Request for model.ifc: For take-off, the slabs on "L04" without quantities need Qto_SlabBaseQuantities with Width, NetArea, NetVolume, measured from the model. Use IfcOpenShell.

First a look at what the model holds.

```python
import ifcopenshell
import ifcopenshell.util.element
import ifcopenshell.util.unit

model = ifcopenshell.open("model.ifc")
print(model.schema)
for unit_type in ("LENGTHUNIT", "AREAUNIT", "VOLUMEUNIT"):
    print(unit_type, ifcopenshell.util.unit.calculate_unit_scale(model, unit_type))
storey = next(s for s in model.by_type("IfcBuildingStorey") if s.Name == "L04")
slabs = [e for e in ifcopenshell.util.element.get_decomposition(storey) if e.is_a("IfcSlab")]
for e in sorted(slabs, key=lambda e: e.id()):
    print(e.id(), e.is_a(), e.Name, list(ifcopenshell.util.element.get_psets(e, qtos_only=True)), sep=" | ")
```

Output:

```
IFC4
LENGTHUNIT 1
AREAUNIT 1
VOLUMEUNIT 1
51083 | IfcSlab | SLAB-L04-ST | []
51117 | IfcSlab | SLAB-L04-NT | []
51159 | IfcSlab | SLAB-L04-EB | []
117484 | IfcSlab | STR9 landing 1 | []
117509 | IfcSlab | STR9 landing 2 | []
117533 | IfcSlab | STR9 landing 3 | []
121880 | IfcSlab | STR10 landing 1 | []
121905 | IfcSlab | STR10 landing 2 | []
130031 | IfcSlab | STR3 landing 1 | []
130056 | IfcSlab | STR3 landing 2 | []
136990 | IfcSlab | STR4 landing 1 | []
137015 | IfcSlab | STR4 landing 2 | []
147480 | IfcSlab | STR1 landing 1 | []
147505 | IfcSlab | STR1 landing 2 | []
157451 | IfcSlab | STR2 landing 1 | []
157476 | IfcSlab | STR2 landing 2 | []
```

```python
import ifcopenshell
import ifcopenshell.api.pset
import ifcopenshell.geom
import ifcopenshell.util.element
import ifcopenshell.util.shape
import ifcopenshell.util.unit

model = ifcopenshell.open("model.ifc")
unit_scale = ifcopenshell.util.unit.calculate_unit_scale(model)
area_scale = ifcopenshell.util.unit.calculate_unit_scale(model, "AREAUNIT")
volume_scale = ifcopenshell.util.unit.calculate_unit_scale(model, "VOLUMEUNIT")
settings = ifcopenshell.geom.settings()

storey = next(s for s in model.by_type("IfcBuildingStorey") if s.Name == "L04")
slabs = [e for e in ifcopenshell.util.element.get_decomposition(storey) if e.is_a("IfcSlab")]

for e in sorted(slabs, key=lambda e: e.id()):
    if ifcopenshell.util.element.get_psets(e, qtos_only=True, should_inherit=False):
        continue
    # Geometry comes back in metres, in the element's own axes.
    shape = ifcopenshell.geom.create_shape(settings, e)
    values = {
        "Width": ifcopenshell.util.shape.get_z(shape.geometry) / unit_scale,
        "NetArea": ifcopenshell.util.shape.get_footprint_area(shape.geometry) / area_scale,
        "NetVolume": ifcopenshell.util.shape.get_volume(shape.geometry) / volume_scale,
    }
    qto = ifcopenshell.api.pset.add_qto(model, product=e, name="Qto_SlabBaseQuantities")
    ifcopenshell.api.pset.edit_qto(model, qto=qto, properties=values)
    print(e.id(), {k: round(v, 3) for k, v in values.items()})

model.write("model-out.ifc")
```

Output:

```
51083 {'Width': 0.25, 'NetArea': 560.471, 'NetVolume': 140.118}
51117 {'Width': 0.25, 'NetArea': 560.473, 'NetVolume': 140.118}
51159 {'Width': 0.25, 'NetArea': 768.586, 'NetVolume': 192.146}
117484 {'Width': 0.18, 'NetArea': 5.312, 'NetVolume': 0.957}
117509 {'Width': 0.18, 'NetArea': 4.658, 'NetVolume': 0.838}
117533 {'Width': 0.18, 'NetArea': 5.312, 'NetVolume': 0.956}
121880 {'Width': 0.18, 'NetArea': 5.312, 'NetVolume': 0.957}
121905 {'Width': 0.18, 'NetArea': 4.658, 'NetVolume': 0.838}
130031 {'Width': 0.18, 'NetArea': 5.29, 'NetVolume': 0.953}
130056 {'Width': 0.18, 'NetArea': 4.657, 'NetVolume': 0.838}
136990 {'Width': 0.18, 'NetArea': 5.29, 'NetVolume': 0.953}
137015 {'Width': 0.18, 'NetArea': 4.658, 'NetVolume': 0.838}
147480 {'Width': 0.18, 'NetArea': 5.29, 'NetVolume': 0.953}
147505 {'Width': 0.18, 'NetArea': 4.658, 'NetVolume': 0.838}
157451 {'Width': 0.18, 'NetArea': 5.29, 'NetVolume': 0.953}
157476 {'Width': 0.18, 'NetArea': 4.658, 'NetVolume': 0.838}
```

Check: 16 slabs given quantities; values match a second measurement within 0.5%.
